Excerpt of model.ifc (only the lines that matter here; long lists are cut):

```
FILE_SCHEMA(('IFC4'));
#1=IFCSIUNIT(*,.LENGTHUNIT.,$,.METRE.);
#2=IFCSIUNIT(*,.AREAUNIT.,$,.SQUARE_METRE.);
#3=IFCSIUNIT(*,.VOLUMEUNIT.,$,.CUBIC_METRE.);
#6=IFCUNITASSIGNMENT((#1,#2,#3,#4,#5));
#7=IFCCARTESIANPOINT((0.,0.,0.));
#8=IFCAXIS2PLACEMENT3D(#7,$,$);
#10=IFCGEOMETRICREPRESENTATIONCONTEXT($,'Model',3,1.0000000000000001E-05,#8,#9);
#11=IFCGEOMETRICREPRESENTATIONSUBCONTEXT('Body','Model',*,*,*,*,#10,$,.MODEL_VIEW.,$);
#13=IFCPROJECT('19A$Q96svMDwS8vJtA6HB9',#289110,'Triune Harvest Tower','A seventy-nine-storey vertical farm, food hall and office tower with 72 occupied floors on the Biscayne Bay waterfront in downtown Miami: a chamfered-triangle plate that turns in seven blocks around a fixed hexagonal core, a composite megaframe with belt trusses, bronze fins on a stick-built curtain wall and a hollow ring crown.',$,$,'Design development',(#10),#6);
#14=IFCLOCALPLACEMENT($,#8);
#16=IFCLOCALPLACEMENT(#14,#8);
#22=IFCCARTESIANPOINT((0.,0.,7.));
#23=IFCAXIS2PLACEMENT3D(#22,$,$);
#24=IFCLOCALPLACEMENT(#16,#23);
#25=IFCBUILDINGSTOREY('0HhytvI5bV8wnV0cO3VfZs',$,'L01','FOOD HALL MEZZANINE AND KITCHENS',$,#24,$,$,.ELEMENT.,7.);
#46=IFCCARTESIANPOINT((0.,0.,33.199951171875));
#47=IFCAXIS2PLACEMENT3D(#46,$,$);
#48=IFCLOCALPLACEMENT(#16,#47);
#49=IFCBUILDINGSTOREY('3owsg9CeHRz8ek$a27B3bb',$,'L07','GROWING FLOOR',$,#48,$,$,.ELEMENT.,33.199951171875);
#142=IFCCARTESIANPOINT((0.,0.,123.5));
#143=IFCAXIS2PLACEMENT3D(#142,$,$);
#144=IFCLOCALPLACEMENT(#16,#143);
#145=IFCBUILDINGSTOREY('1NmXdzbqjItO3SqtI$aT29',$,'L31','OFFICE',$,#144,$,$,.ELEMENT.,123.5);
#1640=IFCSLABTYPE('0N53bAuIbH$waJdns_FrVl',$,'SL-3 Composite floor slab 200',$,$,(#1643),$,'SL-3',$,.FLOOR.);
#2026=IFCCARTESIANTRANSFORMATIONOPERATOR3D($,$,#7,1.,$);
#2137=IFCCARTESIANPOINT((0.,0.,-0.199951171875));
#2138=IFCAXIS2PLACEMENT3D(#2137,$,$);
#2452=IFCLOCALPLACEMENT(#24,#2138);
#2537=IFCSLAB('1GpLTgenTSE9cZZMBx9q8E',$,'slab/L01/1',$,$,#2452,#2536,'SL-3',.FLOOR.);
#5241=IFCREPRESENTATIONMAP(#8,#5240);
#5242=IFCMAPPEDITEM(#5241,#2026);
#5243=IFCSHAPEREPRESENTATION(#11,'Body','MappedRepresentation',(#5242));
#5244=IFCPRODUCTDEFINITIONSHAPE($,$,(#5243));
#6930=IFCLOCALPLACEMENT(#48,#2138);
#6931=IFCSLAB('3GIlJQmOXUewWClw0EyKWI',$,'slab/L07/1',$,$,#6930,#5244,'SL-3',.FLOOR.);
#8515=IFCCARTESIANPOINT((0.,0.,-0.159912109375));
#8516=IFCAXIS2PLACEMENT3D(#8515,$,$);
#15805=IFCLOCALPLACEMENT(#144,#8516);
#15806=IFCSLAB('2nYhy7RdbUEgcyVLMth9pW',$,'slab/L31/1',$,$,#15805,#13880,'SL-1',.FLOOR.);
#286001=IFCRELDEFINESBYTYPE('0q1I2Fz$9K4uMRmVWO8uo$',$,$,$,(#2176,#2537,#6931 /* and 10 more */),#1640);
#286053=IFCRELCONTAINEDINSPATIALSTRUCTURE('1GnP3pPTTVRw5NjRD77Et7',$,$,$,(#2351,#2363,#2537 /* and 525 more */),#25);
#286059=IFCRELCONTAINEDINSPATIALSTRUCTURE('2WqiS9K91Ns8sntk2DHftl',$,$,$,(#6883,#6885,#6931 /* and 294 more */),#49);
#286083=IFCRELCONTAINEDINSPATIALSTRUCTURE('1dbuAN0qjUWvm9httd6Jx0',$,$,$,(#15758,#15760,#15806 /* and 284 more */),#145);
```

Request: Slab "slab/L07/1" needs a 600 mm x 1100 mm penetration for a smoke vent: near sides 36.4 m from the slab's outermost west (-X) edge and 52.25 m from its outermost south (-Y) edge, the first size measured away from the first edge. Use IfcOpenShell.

```python
import numpy as np
import ifcopenshell
import ifcopenshell.api.feature
import ifcopenshell.api.geometry
import ifcopenshell.api.root
import ifcopenshell.geom
import ifcopenshell.util.placement
import ifcopenshell.util.representation
import ifcopenshell.util.shape
import ifcopenshell.util.unit

model = ifcopenshell.open("model.ifc")
unit_scale = ifcopenshell.util.unit.calculate_unit_scale(model)
settings = ifcopenshell.geom.settings()


def volume(element):
    """Net volume in cubic metres, openings subtracted."""
    shape = ifcopenshell.geom.create_shape(settings, element)
    return ifcopenshell.util.shape.get_volume(shape.geometry)


slab = model.by_guid("3GIlJQmOXUewWClw0EyKWI")
before = volume(slab)

# Extent in the slab's own axes, in metres. The edges named are its -X and -Y sides.
slab_shape = ifcopenshell.geom.create_shape(settings, slab)
vertices = ifcopenshell.util.shape.get_vertices(slab_shape.geometry)
x_min, y_min, bottom = vertices.min(axis=0)
top = vertices[:, 2].max()

opening = ifcopenshell.api.root.create_entity(model, ifc_class="IfcOpeningElement", name="Smoke vent opening", predefined_type="OPENING")
context = ifcopenshell.util.representation.get_context(model, "Model", "Body", "MODEL_VIEW")
width, depth = 0.6, 1.1
outline = [(0.0, 0.0), (width, 0.0), (width, depth), (0.0, depth), (0.0, 0.0)]
# Overshoot both faces by 50 mm so the cut is clean.
shape = ifcopenshell.api.geometry.add_slab_representation(
    model, context=context, depth=top - bottom + 0.1, polyline=outline
)
ifcopenshell.api.geometry.assign_representation(model, product=opening, representation=shape)

matrix = ifcopenshell.util.placement.get_local_placement(slab.ObjectPlacement)
matrix[:, 3] = matrix @ np.append(np.array([x_min + 36.4, y_min + 52.25, bottom - 0.05]) / unit_scale, 1.0)
ifcopenshell.api.geometry.edit_object_placement(model, product=opening, matrix=matrix, is_si=False)
ifcopenshell.api.feature.add_feature(model, feature=opening, element=slab)

after = volume(slab)

print(f"slab volume {before:.3f} -> {after:.3f} m3")

model.write("model_v2.ifc")
```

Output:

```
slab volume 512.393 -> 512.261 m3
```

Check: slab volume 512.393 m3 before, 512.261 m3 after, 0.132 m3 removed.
